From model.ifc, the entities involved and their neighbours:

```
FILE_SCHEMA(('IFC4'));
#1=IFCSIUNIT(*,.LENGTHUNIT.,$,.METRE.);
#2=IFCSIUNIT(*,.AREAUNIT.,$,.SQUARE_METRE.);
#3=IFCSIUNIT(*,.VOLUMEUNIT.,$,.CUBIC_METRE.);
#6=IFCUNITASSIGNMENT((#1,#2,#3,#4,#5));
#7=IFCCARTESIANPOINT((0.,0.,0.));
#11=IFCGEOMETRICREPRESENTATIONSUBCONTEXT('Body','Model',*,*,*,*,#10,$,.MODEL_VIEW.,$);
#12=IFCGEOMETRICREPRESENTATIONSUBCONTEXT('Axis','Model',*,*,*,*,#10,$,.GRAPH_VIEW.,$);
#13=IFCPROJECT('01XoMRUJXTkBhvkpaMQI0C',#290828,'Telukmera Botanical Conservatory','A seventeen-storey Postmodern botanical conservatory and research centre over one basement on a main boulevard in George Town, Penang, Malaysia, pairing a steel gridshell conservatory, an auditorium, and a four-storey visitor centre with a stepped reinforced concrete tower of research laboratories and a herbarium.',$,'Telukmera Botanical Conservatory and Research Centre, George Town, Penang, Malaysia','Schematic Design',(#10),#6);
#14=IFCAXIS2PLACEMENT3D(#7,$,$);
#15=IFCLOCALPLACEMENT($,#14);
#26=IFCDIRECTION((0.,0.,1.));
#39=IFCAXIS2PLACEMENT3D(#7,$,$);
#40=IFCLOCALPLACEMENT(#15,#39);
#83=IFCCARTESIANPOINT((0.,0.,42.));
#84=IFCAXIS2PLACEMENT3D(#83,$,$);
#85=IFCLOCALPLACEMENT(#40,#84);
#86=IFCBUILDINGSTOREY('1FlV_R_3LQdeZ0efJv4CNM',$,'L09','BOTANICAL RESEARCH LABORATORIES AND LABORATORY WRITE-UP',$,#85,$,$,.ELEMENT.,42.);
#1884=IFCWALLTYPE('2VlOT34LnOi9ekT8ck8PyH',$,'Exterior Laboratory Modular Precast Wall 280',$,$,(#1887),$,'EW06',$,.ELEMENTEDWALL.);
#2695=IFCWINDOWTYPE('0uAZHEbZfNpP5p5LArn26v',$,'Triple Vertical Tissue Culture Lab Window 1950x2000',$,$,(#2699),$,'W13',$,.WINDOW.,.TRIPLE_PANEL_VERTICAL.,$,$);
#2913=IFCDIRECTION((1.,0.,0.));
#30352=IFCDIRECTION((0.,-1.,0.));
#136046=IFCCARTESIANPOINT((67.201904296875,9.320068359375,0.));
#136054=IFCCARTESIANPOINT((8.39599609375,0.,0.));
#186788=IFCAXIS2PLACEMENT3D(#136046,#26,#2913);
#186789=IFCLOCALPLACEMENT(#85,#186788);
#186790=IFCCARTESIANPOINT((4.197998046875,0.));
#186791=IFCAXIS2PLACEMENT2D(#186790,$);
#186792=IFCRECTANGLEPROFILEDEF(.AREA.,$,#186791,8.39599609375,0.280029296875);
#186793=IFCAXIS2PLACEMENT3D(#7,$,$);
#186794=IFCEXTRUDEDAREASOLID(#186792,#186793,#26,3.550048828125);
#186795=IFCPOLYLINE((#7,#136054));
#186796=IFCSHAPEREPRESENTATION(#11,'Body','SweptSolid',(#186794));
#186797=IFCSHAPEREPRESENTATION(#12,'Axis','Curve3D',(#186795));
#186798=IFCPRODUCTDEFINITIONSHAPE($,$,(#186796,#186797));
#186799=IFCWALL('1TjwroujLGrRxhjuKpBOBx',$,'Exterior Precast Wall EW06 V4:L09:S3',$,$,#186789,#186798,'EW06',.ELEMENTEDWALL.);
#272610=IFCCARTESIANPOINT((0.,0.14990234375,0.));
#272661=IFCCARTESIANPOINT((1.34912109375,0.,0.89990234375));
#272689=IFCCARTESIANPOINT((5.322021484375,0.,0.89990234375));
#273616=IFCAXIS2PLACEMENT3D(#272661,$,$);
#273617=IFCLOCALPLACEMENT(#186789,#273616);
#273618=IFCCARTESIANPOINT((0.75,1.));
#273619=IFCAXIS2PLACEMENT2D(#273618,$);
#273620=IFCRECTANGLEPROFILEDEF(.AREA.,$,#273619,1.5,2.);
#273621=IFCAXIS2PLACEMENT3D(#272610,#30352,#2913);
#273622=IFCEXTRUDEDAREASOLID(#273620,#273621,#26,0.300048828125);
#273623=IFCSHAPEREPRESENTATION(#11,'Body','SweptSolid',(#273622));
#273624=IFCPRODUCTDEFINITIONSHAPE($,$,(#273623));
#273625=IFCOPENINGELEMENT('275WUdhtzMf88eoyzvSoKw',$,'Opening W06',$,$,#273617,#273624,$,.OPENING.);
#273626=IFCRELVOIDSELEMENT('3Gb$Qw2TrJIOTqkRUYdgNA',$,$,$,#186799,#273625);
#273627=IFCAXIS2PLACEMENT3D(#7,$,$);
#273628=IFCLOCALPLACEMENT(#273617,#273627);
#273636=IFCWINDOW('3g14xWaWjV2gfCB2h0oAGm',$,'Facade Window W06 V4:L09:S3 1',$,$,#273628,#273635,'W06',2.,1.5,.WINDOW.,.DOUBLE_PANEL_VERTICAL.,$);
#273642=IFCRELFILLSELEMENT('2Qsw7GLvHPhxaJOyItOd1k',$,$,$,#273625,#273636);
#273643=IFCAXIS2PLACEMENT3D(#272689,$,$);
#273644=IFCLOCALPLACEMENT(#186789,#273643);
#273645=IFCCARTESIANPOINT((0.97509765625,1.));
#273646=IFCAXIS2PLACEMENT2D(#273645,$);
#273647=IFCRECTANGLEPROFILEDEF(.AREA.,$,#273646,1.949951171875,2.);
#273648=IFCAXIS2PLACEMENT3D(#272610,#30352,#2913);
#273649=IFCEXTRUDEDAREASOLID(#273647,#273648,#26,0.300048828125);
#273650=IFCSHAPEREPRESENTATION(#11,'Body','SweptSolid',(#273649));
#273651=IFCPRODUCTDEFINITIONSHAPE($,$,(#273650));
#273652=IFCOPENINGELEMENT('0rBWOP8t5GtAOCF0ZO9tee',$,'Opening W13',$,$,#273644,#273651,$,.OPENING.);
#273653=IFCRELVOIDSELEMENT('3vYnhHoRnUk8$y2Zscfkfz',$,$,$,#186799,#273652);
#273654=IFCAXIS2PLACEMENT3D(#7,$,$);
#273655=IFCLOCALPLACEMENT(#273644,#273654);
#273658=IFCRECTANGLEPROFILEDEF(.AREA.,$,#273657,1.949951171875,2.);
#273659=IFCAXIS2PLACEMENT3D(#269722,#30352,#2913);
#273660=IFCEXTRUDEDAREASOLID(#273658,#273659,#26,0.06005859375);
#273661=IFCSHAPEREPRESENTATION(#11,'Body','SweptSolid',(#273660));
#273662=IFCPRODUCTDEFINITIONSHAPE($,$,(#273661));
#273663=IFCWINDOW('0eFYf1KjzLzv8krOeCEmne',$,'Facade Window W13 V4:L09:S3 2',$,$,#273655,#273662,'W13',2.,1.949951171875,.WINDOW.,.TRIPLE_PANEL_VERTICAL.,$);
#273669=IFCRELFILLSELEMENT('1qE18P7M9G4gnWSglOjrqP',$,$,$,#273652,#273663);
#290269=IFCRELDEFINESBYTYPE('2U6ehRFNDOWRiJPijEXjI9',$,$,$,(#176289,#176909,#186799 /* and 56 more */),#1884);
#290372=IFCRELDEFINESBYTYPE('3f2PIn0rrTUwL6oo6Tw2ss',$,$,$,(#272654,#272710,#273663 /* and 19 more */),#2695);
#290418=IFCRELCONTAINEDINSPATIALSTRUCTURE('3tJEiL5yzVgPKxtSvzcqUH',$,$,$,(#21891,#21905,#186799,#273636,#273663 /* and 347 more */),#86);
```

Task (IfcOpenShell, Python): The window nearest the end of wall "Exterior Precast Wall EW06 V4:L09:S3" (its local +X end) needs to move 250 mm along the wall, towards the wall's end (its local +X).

```python
import ifcopenshell
import ifcopenshell.api.geometry
import ifcopenshell.util.placement
import ifcopenshell.util.unit

model = ifcopenshell.open("model.ifc")
unit_scale = ifcopenshell.util.unit.calculate_unit_scale(model)

window = model.by_guid("0eFYf1KjzLzv8krOeCEmne")
opening = window.FillsVoids[0].RelatingOpeningElement
wall = opening.VoidsElements[0].RelatingBuildingElement

wall_matrix = ifcopenshell.util.placement.get_local_placement(wall.ObjectPlacement)
shift = wall_matrix[:3, 0] * 0.25 / unit_scale
before = ifcopenshell.util.placement.get_local_placement(window.ObjectPlacement)[:3, 3].copy()

# The window is placed relative to its opening, so it follows when the opening moves.
matrix = ifcopenshell.util.placement.get_local_placement(opening.ObjectPlacement)
matrix[:3, 3] += shift
ifcopenshell.api.geometry.edit_object_placement(
    model, product=opening, matrix=matrix, is_si=False, should_transform_children=True
)

after = ifcopenshell.util.placement.get_local_placement(window.ObjectPlacement)[:3, 3]
print("window moved by", (after - before).round(3) + 0.0)

model.write("model_updated.ifc")
```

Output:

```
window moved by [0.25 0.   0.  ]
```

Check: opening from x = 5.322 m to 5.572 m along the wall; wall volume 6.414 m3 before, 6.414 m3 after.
